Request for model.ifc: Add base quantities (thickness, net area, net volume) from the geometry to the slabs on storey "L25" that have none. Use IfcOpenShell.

First a look at what the model holds.

```python
import ifcopenshell
import ifcopenshell.util.element
import ifcopenshell.util.unit

model = ifcopenshell.open("model.ifc")
print(model.schema)
for unit_type in ("LENGTHUNIT", "AREAUNIT", "VOLUMEUNIT"):
    print(unit_type, ifcopenshell.util.unit.calculate_unit_scale(model, unit_type))
storey = next(s for s in model.by_type("IfcBuildingStorey") if s.Name == "L25")
slabs = [e for e in ifcopenshell.util.element.get_decomposition(storey) if e.is_a("IfcSlab")]
for e in sorted(slabs, key=lambda e: e.id()):
    print(e.id(), e.is_a(), e.Name, list(ifcopenshell.util.element.get_psets(e, qtos_only=True)), sep=" | ")
```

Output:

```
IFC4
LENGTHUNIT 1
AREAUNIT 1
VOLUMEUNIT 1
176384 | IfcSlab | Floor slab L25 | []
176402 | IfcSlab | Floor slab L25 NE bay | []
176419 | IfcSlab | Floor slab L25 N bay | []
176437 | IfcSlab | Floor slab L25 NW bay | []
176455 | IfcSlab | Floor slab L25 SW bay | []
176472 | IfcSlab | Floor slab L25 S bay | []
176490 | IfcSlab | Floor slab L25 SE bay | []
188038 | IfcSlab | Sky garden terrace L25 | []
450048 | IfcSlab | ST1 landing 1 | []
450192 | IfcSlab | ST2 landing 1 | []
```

```python
import ifcopenshell
import ifcopenshell.api.pset
import ifcopenshell.geom
import ifcopenshell.util.element
import ifcopenshell.util.shape
import ifcopenshell.util.unit

model = ifcopenshell.open("model.ifc")
unit_scale = ifcopenshell.util.unit.calculate_unit_scale(model)
area_scale = ifcopenshell.util.unit.calculate_unit_scale(model, "AREAUNIT")
volume_scale = ifcopenshell.util.unit.calculate_unit_scale(model, "VOLUMEUNIT")
settings = ifcopenshell.geom.settings()

storey = next(s for s in model.by_type("IfcBuildingStorey") if s.Name == "L25")
slabs = [e for e in ifcopenshell.util.element.get_decomposition(storey) if e.is_a("IfcSlab")]

for e in sorted(slabs, key=lambda e: e.id()):
    if ifcopenshell.util.element.get_psets(e, qtos_only=True, should_inherit=False):
        continue
    # Geometry comes back in metres, in the element's own axes.
    shape = ifcopenshell.geom.create_shape(settings, e)
    values = {
        "Width": ifcopenshell.util.shape.get_z(shape.geometry) / unit_scale,
        "NetArea": ifcopenshell.util.shape.get_footprint_area(shape.geometry) / area_scale,
        "NetVolume": ifcopenshell.util.shape.get_volume(shape.geometry) / volume_scale,
    }
    qto = ifcopenshell.api.pset.add_qto(model, product=e, name="Qto_SlabBaseQuantities")
    ifcopenshell.api.pset.edit_qto(model, qto=qto, properties=values)
    print(e.id(), {k: round(v, 3) for k, v in values.items()})

model.write("model_rev.ifc")
```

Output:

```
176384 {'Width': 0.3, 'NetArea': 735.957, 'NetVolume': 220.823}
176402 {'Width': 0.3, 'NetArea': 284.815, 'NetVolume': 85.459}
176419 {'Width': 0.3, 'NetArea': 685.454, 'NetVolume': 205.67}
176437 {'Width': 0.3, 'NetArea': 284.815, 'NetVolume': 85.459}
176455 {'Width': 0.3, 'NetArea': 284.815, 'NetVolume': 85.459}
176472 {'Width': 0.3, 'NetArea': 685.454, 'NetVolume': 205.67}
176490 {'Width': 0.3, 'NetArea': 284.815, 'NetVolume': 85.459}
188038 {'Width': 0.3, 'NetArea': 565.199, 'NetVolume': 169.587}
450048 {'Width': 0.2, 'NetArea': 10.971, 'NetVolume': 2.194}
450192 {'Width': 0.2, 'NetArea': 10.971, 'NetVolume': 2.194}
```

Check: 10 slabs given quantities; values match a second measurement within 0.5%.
